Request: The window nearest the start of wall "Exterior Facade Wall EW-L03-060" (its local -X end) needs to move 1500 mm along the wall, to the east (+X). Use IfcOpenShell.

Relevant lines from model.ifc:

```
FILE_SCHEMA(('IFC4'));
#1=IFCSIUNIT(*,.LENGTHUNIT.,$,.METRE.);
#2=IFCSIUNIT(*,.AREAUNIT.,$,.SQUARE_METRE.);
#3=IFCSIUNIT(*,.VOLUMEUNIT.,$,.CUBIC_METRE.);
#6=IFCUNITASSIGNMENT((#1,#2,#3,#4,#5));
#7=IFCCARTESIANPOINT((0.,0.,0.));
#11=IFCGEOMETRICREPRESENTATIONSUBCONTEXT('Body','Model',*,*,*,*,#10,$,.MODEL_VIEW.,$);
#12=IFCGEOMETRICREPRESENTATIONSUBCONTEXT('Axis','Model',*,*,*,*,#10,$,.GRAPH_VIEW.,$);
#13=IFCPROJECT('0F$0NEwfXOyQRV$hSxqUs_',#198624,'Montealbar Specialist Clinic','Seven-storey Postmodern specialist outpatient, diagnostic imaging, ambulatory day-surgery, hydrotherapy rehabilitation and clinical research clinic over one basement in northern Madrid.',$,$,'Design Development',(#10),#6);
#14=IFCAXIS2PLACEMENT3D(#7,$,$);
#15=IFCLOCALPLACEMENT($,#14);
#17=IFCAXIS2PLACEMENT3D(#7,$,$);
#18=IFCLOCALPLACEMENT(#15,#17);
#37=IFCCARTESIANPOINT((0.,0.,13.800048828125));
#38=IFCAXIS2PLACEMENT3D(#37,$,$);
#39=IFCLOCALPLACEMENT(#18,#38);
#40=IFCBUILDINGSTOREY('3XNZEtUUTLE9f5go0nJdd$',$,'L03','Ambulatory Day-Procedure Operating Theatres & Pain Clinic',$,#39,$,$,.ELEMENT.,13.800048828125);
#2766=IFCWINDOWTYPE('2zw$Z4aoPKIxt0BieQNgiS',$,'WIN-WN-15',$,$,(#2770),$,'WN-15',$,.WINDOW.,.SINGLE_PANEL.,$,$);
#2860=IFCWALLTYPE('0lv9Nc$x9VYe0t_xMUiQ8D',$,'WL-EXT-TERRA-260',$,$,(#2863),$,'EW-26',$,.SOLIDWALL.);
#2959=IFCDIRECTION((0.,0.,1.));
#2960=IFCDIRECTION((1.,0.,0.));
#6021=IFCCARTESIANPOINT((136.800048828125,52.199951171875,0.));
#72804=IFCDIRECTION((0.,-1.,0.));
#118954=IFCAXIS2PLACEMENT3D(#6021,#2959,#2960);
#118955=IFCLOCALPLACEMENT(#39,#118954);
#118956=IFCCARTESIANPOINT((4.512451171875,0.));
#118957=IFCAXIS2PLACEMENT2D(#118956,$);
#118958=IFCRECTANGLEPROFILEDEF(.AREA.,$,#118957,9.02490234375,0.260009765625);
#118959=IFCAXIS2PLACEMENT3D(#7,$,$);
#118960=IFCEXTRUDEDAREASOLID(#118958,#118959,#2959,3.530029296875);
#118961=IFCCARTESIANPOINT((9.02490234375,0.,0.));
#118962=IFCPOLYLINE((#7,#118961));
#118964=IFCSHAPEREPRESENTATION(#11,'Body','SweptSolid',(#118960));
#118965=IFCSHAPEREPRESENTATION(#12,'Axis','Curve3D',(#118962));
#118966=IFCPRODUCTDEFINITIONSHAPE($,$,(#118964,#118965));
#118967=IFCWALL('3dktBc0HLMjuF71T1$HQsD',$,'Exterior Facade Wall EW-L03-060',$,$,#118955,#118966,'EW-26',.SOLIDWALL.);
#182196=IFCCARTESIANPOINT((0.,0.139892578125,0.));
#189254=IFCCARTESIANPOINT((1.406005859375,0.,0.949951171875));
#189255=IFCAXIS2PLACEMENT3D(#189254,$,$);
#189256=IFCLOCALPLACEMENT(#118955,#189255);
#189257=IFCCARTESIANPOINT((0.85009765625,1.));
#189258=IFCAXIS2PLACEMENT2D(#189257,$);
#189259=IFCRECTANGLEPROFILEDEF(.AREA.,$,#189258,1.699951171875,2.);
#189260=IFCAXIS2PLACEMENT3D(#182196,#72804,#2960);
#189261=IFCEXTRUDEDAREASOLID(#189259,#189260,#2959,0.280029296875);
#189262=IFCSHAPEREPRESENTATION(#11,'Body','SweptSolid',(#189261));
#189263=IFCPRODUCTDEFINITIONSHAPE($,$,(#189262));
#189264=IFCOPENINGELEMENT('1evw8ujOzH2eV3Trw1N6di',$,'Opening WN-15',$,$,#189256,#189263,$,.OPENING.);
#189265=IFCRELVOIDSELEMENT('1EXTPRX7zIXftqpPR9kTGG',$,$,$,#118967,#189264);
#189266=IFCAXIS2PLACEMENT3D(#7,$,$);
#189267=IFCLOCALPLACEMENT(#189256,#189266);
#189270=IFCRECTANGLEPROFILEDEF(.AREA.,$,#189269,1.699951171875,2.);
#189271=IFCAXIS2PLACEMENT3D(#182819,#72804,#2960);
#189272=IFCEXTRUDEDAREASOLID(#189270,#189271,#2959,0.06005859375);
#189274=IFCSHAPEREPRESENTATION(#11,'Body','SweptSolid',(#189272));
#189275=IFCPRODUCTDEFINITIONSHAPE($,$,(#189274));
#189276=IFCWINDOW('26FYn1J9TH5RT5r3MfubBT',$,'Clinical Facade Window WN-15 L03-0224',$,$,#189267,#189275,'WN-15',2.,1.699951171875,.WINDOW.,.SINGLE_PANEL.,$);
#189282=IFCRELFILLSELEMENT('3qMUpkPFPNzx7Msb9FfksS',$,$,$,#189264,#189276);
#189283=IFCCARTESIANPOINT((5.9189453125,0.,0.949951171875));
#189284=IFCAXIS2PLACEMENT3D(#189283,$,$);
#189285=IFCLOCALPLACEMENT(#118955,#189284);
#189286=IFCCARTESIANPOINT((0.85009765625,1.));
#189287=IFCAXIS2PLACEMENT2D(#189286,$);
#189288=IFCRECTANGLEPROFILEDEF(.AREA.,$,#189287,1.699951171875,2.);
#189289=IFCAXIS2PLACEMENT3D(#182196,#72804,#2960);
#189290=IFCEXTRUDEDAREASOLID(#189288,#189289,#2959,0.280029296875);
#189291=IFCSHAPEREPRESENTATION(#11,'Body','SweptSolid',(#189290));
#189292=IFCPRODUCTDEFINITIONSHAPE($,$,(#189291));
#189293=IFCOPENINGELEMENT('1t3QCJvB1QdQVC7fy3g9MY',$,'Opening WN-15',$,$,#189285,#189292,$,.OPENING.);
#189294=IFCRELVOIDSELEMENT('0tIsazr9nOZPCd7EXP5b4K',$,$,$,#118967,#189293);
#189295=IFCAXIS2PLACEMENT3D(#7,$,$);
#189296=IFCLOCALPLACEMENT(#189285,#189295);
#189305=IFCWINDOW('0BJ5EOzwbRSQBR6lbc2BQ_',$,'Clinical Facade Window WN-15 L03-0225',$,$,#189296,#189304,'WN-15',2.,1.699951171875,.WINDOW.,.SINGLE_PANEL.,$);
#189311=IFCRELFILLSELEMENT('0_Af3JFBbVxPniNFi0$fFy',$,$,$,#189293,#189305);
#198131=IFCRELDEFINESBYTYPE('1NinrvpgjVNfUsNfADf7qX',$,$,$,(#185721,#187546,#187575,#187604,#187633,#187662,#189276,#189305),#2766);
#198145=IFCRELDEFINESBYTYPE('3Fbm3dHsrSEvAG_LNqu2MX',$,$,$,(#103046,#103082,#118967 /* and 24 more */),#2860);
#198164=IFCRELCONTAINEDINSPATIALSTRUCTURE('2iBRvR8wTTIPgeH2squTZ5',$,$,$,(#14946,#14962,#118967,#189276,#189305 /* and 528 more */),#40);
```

```python
import ifcopenshell
import ifcopenshell.api.geometry
import ifcopenshell.util.placement
import ifcopenshell.util.unit

model = ifcopenshell.open("model.ifc")
unit_scale = ifcopenshell.util.unit.calculate_unit_scale(model)

window = model.by_guid("26FYn1J9TH5RT5r3MfubBT")
opening = window.FillsVoids[0].RelatingOpeningElement
wall = opening.VoidsElements[0].RelatingBuildingElement

wall_matrix = ifcopenshell.util.placement.get_local_placement(wall.ObjectPlacement)
shift = wall_matrix[:3, 0] * 1.5 / unit_scale
before = ifcopenshell.util.placement.get_local_placement(window.ObjectPlacement)[:3, 3].copy()

# The window is placed relative to its opening, so it follows when the opening moves.
matrix = ifcopenshell.util.placement.get_local_placement(opening.ObjectPlacement)
matrix[:3, 3] += shift
ifcopenshell.api.geometry.edit_object_placement(
    model, product=opening, matrix=matrix, is_si=False, should_transform_children=True
)

after = ifcopenshell.util.placement.get_local_placement(window.ObjectPlacement)[:3, 3]
print("window moved by", (after - before).round(3) + 0.0)

model.write("model_v2.ifc")
```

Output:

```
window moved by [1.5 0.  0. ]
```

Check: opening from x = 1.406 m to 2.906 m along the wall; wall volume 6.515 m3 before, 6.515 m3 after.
